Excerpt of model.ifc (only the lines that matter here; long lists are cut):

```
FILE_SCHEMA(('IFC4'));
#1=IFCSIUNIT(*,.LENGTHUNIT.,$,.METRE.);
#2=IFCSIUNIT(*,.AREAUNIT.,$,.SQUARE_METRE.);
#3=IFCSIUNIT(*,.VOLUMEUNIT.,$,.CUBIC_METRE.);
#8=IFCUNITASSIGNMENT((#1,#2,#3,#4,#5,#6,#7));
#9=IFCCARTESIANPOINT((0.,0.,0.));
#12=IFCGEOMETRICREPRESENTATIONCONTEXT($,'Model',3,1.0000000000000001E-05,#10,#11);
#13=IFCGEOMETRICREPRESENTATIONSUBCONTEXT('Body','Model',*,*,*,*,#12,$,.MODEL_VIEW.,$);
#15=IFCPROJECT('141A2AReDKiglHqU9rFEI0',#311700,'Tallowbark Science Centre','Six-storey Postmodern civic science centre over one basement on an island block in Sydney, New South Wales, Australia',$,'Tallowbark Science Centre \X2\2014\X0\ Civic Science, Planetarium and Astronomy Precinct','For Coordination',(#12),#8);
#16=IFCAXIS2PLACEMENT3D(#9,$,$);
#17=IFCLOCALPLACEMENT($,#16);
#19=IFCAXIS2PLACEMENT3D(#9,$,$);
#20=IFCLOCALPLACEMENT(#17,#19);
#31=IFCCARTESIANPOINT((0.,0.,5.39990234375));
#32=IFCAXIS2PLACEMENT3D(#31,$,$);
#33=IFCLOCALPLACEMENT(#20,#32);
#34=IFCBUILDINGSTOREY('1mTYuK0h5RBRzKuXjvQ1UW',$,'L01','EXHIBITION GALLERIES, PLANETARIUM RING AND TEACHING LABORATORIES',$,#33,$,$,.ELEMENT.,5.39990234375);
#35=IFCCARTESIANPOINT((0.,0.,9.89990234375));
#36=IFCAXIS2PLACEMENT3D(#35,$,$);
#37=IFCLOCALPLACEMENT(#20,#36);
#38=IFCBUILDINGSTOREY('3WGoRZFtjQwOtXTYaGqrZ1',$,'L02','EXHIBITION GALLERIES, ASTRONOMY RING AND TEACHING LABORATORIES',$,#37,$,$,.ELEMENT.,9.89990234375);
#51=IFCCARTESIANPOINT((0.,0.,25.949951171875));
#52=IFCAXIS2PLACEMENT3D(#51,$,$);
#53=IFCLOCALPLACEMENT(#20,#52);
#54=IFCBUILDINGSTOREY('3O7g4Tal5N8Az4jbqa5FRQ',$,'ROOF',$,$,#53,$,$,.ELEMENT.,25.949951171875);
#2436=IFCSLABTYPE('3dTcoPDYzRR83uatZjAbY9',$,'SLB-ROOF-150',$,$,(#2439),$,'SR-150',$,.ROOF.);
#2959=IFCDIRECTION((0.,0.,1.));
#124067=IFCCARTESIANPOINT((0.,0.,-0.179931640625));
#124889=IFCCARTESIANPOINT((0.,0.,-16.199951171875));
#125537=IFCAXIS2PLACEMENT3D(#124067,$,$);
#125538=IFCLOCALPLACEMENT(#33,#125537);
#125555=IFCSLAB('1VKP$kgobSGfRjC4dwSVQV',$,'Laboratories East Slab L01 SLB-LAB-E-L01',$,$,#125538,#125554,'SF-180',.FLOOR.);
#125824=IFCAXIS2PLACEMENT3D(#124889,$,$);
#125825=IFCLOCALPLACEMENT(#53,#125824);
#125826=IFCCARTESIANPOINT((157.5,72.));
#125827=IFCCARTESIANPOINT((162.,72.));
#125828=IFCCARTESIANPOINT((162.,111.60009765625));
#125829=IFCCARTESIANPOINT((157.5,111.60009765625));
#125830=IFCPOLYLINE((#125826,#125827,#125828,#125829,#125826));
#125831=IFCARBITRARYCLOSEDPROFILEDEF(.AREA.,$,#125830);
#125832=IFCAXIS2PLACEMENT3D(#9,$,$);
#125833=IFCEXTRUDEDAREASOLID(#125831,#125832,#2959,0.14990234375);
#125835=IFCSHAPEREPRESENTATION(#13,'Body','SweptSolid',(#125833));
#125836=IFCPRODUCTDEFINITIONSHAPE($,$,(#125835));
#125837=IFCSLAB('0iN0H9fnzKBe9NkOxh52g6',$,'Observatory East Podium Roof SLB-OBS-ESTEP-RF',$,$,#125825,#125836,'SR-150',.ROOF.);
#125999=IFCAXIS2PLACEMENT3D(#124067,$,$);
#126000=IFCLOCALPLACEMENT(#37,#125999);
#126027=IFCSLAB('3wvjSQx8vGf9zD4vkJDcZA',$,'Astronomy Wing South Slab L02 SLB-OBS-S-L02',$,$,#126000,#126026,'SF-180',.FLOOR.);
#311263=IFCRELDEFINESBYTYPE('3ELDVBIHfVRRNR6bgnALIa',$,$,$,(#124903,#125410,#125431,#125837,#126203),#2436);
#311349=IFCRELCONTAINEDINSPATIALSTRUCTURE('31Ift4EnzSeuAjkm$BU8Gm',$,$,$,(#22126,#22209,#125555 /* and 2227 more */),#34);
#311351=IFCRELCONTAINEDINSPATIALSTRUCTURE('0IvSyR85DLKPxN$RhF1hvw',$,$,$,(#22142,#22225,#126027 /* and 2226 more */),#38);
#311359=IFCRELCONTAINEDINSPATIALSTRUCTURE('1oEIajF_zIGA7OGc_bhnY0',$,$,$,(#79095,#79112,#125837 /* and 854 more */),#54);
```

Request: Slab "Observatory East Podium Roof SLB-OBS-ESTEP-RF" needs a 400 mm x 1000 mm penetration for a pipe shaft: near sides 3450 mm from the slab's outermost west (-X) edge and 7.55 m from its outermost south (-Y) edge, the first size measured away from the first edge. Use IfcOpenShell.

```python
import numpy as np
import ifcopenshell
import ifcopenshell.api.feature
import ifcopenshell.api.geometry
import ifcopenshell.api.root
import ifcopenshell.geom
import ifcopenshell.util.placement
import ifcopenshell.util.representation
import ifcopenshell.util.shape
import ifcopenshell.util.unit

model = ifcopenshell.open("model.ifc")
unit_scale = ifcopenshell.util.unit.calculate_unit_scale(model)
settings = ifcopenshell.geom.settings()


def volume(element):
    """Net volume in cubic metres, openings subtracted."""
    shape = ifcopenshell.geom.create_shape(settings, element)
    return ifcopenshell.util.shape.get_volume(shape.geometry)


slab = model.by_guid("0iN0H9fnzKBe9NkOxh52g6")
before = volume(slab)

# Extent in the slab's own axes, in metres. The edges named are its -X and -Y sides.
slab_shape = ifcopenshell.geom.create_shape(settings, slab)
vertices = ifcopenshell.util.shape.get_vertices(slab_shape.geometry)
x_min, y_min, bottom = vertices.min(axis=0)
top = vertices[:, 2].max()

opening = ifcopenshell.api.root.create_entity(model, ifc_class="IfcOpeningElement", name="Pipe shaft opening", predefined_type="OPENING")
context = ifcopenshell.util.representation.get_context(model, "Model", "Body", "MODEL_VIEW")
width, depth = 0.4, 1
outline = [(0.0, 0.0), (width, 0.0), (width, depth), (0.0, depth), (0.0, 0.0)]
# Overshoot both faces by 50 mm so the cut is clean.
shape = ifcopenshell.api.geometry.add_slab_representation(
    model, context=context, depth=top - bottom + 0.1, polyline=outline
)
ifcopenshell.api.geometry.assign_representation(model, product=opening, representation=shape)

matrix = ifcopenshell.util.placement.get_local_placement(slab.ObjectPlacement)
matrix[:, 3] = matrix @ np.append(np.array([x_min + 3.45, y_min + 7.55, bottom - 0.05]) / unit_scale, 1.0)
ifcopenshell.api.geometry.edit_object_placement(model, product=opening, matrix=matrix, is_si=False)
ifcopenshell.api.feature.add_feature(model, feature=opening, element=slab)

after = volume(slab)

print(f"slab volume {before:.3f} -> {after:.3f} m3")

model.write("model-out.ifc")
```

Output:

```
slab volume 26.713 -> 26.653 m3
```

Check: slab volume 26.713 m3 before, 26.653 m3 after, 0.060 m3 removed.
